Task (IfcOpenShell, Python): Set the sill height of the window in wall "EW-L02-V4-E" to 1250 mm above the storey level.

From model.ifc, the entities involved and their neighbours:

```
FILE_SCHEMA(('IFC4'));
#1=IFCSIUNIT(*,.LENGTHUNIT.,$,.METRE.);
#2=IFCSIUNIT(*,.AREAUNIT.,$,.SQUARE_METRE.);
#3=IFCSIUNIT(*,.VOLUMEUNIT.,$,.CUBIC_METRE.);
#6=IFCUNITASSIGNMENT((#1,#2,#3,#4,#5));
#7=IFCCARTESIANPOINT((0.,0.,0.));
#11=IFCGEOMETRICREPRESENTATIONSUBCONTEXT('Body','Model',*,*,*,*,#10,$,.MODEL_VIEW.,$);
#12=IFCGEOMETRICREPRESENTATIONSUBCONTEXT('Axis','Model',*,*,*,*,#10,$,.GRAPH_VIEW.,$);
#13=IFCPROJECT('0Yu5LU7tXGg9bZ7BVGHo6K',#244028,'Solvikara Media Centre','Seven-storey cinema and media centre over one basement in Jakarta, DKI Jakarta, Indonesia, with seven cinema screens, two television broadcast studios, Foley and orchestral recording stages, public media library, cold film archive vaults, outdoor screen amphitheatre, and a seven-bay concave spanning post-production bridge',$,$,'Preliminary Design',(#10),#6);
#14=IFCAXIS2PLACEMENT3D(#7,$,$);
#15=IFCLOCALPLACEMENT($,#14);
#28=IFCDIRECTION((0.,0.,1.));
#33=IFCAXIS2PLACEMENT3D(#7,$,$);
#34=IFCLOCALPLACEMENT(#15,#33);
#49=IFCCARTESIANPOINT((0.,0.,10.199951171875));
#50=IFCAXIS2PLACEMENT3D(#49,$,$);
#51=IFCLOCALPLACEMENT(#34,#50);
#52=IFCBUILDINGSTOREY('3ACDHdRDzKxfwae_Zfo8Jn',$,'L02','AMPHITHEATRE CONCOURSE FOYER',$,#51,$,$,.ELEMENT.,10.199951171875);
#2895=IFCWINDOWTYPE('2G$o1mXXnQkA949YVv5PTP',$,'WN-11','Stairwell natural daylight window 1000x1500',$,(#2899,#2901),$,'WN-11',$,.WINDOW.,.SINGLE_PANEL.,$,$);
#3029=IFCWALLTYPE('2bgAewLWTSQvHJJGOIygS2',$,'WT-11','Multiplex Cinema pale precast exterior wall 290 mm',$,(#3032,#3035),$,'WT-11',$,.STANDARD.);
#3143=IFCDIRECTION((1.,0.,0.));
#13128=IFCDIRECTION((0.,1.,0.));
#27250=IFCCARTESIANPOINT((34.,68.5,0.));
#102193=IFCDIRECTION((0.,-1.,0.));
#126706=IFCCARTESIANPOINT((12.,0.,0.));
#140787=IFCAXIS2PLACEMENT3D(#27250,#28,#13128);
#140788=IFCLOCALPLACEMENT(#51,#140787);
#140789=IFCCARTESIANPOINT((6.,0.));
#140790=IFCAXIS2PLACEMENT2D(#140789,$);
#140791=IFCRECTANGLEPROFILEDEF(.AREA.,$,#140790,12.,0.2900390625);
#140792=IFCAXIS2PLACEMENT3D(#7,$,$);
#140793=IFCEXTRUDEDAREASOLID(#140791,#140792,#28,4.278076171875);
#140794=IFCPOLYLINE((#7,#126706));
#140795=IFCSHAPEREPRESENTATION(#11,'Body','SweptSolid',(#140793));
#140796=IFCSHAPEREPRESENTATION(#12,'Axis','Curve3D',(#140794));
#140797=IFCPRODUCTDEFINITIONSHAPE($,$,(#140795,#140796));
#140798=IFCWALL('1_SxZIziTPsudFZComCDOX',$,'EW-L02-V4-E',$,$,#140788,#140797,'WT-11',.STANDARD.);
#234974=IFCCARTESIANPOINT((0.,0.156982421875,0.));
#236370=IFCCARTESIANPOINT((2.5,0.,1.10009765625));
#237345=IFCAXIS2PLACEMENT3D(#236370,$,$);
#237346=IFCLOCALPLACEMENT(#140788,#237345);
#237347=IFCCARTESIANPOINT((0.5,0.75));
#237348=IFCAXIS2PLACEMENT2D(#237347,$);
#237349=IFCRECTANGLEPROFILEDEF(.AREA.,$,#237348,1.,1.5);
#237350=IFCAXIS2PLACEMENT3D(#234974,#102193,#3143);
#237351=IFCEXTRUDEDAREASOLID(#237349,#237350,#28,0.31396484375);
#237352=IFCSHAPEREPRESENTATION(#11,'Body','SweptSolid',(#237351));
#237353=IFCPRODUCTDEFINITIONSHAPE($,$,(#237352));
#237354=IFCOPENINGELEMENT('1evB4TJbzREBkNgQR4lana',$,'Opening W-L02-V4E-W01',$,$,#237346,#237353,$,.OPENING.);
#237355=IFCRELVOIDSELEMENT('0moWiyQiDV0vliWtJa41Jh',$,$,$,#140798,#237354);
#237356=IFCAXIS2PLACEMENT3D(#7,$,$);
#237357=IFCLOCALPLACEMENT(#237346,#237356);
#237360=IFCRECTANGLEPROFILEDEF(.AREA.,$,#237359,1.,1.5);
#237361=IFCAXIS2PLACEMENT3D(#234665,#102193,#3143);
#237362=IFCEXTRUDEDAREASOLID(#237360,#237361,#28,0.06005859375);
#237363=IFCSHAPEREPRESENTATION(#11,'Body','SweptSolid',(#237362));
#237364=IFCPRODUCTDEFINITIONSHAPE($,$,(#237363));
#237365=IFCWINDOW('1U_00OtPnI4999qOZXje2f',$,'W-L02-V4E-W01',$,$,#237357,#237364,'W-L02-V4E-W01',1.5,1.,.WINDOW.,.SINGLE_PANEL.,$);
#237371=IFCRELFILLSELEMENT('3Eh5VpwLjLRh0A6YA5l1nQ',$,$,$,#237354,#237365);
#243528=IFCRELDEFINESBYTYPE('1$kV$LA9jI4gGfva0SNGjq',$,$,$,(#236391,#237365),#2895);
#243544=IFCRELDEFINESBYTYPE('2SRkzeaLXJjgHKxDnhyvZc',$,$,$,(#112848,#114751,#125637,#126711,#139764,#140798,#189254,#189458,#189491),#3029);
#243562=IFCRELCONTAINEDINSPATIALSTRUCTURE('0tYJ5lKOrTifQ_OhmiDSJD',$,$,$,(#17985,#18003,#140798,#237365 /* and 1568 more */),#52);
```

```python
import numpy as np
import ifcopenshell
import ifcopenshell.api.geometry
import ifcopenshell.geom
import ifcopenshell.util.element
import ifcopenshell.util.placement
import ifcopenshell.util.shape
import ifcopenshell.util.unit

model = ifcopenshell.open("model.ifc")
unit_scale = ifcopenshell.util.unit.calculate_unit_scale(model)

window = model.by_id(237365)
opening = window.FillsVoids[0].RelatingOpeningElement
storey = ifcopenshell.util.element.get_container(window, ifc_class="IfcBuildingStorey")
level = ifcopenshell.util.placement.get_local_placement(storey.ObjectPlacement)[2, 3]

# The opening's origin need not be at the sill, so measure its lowest point.
shape = ifcopenshell.geom.create_shape(ifcopenshell.geom.settings(), opening)
bottom = ifcopenshell.util.shape.get_shape_bottom_elevation(shape, shape.geometry) / unit_scale
dz = level + 1.25 - bottom

shift = np.array([0.0, 0.0, dz])
# The window is placed relative to its opening, so it follows when the opening moves.
matrix = ifcopenshell.util.placement.get_local_placement(opening.ObjectPlacement)
matrix[:3, 3] += shift
ifcopenshell.api.geometry.edit_object_placement(
    model, product=opening, matrix=matrix, is_si=False, should_transform_children=True
)

print(f"moved by {dz * unit_scale:+.3f} m")

model.write("model_updated.ifc")
```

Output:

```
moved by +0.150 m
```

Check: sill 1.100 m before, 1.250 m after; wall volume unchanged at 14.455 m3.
